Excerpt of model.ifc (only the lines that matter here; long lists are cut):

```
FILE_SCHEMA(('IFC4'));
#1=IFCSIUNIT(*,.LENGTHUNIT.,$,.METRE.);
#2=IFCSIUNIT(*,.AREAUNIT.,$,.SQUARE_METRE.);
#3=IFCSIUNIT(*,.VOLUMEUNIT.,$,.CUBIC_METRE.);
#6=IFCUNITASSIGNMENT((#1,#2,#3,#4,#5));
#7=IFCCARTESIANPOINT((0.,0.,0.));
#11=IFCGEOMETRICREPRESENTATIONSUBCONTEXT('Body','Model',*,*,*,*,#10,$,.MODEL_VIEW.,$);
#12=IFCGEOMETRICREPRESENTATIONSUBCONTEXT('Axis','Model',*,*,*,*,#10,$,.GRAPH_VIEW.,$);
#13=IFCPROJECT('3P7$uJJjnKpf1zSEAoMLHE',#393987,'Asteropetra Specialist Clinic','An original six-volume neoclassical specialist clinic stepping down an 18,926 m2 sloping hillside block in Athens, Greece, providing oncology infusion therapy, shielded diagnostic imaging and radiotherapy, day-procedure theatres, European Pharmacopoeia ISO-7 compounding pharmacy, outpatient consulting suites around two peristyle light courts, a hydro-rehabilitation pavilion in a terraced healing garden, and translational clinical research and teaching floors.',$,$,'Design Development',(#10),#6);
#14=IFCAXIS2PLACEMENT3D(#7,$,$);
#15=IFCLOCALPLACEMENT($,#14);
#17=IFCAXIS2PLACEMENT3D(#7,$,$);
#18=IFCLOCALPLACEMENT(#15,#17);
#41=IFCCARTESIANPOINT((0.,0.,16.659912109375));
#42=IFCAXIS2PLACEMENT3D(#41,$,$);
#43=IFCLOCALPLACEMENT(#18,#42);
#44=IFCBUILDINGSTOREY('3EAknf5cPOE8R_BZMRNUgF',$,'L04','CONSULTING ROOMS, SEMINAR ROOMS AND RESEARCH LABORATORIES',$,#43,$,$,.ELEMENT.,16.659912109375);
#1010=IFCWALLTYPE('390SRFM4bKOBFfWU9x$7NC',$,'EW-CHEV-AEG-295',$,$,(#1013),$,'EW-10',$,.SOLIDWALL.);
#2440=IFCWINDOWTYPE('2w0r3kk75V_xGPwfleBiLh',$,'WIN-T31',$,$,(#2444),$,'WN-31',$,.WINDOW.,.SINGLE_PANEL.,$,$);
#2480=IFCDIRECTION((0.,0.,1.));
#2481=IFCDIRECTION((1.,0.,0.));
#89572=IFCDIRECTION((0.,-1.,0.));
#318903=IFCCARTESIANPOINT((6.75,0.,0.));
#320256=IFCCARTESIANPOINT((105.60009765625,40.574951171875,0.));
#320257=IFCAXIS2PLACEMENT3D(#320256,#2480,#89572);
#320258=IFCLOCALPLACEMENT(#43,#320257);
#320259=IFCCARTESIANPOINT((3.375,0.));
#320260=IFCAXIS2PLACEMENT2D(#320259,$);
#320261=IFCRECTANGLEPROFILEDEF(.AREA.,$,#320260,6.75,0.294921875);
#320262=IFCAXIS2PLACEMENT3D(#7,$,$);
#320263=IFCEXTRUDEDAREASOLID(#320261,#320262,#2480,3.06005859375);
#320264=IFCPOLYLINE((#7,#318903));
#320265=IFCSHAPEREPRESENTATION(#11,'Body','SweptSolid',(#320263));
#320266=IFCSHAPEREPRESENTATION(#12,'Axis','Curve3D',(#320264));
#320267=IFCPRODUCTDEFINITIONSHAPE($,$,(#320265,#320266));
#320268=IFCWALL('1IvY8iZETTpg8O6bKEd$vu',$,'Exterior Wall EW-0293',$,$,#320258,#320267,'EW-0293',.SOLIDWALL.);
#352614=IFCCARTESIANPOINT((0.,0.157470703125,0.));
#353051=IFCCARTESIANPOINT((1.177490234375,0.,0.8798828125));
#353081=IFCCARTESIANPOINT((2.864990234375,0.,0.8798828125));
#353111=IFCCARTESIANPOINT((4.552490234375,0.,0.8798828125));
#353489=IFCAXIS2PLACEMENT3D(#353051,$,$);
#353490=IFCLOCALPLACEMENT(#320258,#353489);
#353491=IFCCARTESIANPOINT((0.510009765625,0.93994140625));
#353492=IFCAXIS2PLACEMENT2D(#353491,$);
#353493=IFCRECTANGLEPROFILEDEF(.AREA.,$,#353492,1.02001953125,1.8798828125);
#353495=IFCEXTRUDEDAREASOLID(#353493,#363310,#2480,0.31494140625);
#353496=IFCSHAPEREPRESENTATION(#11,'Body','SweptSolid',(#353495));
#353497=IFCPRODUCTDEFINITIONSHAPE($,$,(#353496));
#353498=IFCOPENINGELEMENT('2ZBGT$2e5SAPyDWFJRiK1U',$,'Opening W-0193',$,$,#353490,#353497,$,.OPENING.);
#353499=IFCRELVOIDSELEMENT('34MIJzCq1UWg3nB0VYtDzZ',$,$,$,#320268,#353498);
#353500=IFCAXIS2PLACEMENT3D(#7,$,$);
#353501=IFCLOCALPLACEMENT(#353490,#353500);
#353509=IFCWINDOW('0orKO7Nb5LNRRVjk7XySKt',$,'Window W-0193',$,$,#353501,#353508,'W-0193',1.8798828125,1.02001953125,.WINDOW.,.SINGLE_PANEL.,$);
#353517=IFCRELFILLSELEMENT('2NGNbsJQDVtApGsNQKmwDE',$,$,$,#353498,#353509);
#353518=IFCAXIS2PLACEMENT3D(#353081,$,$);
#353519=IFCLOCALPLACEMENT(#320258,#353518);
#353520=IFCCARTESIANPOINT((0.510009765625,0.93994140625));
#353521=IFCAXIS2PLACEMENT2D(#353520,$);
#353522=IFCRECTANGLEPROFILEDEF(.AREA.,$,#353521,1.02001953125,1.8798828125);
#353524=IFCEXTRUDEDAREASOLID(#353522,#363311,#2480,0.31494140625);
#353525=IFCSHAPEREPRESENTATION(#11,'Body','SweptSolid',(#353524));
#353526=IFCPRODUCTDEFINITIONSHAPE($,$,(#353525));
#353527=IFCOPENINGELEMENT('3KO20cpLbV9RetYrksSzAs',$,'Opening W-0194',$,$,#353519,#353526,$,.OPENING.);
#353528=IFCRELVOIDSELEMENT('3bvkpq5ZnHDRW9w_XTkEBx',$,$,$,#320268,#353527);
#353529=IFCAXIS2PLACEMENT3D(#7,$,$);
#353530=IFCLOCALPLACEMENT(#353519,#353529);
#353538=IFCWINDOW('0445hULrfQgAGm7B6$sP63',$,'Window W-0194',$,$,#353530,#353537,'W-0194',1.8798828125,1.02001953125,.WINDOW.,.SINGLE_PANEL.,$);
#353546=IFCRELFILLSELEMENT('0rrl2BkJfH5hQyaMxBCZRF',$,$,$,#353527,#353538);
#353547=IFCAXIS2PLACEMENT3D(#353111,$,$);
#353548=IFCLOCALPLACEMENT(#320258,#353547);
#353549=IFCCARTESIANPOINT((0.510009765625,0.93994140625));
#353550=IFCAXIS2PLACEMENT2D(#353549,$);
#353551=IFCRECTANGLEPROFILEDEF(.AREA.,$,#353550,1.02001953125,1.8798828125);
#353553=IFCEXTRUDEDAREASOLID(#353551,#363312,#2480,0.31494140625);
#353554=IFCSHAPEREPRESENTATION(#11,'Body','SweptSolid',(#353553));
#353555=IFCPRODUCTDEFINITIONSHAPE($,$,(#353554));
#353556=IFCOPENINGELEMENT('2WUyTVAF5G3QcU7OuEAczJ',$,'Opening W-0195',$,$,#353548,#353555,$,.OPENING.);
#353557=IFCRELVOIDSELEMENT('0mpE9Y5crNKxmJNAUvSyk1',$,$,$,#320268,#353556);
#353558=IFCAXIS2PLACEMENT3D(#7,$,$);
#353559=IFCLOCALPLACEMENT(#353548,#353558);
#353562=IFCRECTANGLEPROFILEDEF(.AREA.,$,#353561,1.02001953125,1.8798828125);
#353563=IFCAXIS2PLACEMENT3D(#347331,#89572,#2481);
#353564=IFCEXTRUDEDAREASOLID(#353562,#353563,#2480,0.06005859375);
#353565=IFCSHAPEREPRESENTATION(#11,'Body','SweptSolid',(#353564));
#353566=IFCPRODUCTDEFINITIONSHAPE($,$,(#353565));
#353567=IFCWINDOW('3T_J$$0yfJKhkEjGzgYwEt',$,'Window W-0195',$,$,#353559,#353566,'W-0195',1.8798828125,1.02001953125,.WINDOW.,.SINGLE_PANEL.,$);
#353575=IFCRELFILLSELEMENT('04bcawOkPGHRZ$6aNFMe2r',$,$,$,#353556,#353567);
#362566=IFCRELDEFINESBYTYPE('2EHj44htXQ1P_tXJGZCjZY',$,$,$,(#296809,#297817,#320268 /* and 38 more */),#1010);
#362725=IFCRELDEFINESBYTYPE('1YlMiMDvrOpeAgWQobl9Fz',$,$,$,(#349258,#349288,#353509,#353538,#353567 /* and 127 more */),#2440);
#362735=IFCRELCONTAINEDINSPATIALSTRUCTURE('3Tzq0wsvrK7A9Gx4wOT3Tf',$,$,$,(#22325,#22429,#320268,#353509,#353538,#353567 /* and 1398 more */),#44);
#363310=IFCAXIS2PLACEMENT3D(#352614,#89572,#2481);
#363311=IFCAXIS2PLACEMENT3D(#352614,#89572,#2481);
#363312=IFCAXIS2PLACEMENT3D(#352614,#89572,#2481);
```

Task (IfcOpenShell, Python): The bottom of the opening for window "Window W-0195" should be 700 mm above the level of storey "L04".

```python
import numpy as np
import ifcopenshell
import ifcopenshell.api.geometry
import ifcopenshell.geom
import ifcopenshell.util.element
import ifcopenshell.util.placement
import ifcopenshell.util.shape
import ifcopenshell.util.unit

model = ifcopenshell.open("model.ifc")
unit_scale = ifcopenshell.util.unit.calculate_unit_scale(model)

window = model.by_guid("3T_J$$0yfJKhkEjGzgYwEt")
opening = window.FillsVoids[0].RelatingOpeningElement
storey = ifcopenshell.util.element.get_container(window, ifc_class="IfcBuildingStorey")
level = ifcopenshell.util.placement.get_local_placement(storey.ObjectPlacement)[2, 3]

# The opening's origin need not be at the sill, so measure its lowest point.
shape = ifcopenshell.geom.create_shape(ifcopenshell.geom.settings(), opening)
bottom = ifcopenshell.util.shape.get_shape_bottom_elevation(shape, shape.geometry) / unit_scale
dz = level + 0.7 / unit_scale - bottom

shift = np.array([0.0, 0.0, dz])
# The window is placed relative to its opening, so it follows when the opening moves.
matrix = ifcopenshell.util.placement.get_local_placement(opening.ObjectPlacement)
matrix[:3, 3] += shift
ifcopenshell.api.geometry.edit_object_placement(
    model, product=opening, matrix=matrix, is_si=False, should_transform_children=True
)

print(f"moved by {dz * unit_scale:+.3f} m")

model.write("model-out.ifc")
```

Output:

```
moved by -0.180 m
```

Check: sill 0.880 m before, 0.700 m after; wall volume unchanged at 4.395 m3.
